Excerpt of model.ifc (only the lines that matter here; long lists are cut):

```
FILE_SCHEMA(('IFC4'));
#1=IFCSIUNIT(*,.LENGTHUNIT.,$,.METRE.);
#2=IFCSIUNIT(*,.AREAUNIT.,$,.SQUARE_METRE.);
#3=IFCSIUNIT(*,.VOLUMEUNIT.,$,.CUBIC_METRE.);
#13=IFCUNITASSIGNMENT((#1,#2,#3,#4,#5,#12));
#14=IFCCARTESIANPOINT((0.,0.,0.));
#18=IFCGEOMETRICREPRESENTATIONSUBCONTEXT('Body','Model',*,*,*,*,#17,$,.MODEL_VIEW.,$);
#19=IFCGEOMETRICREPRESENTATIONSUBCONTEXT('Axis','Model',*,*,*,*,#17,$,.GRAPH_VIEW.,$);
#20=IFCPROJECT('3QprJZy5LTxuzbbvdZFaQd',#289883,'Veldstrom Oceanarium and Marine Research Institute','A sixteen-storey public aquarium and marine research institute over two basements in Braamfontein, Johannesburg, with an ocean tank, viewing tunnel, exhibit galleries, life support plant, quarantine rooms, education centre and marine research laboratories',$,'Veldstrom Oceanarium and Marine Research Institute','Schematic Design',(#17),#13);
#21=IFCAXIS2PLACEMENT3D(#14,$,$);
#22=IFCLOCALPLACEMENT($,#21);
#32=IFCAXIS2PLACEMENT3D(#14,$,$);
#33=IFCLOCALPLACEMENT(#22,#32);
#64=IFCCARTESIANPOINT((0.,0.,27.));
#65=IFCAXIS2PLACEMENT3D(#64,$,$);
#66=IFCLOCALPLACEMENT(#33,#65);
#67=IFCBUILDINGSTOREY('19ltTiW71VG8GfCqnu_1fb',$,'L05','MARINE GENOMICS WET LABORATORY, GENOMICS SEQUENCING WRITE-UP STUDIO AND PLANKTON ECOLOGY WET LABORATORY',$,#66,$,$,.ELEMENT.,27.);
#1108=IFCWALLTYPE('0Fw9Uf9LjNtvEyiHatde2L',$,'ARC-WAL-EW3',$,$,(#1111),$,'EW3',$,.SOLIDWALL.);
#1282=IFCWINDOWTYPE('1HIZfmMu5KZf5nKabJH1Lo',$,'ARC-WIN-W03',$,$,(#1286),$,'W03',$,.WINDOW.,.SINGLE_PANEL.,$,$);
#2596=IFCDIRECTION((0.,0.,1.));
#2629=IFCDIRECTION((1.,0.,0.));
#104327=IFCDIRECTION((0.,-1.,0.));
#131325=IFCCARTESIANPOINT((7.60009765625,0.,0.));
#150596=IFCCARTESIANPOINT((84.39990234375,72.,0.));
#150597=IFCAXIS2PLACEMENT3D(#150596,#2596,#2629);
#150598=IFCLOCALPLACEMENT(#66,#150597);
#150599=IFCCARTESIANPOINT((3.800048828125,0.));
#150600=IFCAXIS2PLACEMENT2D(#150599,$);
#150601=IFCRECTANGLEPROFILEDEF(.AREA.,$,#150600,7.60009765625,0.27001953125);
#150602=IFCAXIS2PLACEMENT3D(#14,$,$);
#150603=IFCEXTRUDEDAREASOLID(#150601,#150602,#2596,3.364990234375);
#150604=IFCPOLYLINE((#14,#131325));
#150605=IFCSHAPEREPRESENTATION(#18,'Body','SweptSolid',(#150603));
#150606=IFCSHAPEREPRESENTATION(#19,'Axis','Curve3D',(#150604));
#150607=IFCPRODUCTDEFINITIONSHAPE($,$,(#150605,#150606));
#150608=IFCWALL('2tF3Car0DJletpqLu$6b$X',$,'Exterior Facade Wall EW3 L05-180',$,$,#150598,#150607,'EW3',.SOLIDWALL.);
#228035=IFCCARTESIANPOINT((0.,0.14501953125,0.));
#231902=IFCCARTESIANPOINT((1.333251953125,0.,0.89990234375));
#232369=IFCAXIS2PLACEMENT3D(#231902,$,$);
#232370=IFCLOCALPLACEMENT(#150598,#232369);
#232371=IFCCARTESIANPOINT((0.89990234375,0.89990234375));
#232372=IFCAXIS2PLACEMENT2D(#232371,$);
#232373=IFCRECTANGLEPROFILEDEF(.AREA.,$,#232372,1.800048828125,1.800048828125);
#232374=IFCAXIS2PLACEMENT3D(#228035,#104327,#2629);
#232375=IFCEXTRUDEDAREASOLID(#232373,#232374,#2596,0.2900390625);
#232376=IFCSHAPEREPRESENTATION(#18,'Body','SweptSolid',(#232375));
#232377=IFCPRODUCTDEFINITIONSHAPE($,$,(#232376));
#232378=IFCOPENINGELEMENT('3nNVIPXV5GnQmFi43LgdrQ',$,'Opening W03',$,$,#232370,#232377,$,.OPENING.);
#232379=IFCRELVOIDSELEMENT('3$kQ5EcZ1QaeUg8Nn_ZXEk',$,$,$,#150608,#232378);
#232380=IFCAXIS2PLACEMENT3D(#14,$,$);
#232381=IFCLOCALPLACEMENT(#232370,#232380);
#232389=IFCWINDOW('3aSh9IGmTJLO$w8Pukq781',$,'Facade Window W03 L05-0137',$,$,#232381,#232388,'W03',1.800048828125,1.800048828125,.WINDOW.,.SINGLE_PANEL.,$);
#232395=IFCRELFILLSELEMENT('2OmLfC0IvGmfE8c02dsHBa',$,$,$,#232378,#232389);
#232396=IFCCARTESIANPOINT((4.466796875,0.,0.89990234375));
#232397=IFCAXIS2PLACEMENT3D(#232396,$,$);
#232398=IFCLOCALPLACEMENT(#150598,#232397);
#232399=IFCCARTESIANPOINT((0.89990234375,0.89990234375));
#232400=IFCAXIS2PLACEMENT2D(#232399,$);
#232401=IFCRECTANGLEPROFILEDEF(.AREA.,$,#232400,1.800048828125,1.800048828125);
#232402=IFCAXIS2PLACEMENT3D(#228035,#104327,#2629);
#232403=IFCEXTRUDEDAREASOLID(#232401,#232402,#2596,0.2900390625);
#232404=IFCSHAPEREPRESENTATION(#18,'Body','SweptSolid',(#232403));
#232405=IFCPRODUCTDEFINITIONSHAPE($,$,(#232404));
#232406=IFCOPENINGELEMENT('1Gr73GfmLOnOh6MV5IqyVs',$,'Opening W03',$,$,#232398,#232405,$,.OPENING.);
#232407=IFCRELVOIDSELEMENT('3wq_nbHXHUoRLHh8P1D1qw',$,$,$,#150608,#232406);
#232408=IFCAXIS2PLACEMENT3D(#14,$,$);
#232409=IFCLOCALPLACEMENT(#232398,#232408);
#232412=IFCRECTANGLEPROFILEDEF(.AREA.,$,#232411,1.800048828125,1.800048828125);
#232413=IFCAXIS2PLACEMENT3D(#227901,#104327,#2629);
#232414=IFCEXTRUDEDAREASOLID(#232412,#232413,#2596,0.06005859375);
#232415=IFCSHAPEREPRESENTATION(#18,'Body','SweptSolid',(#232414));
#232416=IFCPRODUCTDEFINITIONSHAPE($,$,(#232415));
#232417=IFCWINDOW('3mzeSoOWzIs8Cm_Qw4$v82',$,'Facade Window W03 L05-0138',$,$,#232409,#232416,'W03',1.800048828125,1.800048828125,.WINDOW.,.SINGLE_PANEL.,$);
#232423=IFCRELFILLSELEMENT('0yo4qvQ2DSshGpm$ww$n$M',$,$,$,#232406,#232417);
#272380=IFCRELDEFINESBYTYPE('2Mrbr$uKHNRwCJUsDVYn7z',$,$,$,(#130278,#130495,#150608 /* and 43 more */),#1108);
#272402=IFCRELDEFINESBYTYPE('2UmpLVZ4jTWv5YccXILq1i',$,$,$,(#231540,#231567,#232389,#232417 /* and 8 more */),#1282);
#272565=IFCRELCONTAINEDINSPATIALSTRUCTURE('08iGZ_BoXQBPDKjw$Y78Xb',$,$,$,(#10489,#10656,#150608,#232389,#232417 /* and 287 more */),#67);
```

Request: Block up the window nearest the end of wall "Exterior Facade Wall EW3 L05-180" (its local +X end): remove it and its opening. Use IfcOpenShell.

```python
import ifcopenshell
import ifcopenshell.api.feature
import ifcopenshell.api.root
import ifcopenshell.geom
import ifcopenshell.util.shape

model = ifcopenshell.open("model.ifc")
settings = ifcopenshell.geom.settings()


def volume(element):
    """Net volume in cubic metres, openings subtracted."""
    shape = ifcopenshell.geom.create_shape(settings, element)
    return ifcopenshell.util.shape.get_volume(shape.geometry)


window = model.by_guid("3mzeSoOWzIs8Cm_Qw4$v82")
opening = window.FillsVoids[0].RelatingOpeningElement
wall = opening.VoidsElements[0].RelatingBuildingElement
before = volume(wall)

ifcopenshell.api.root.remove_product(model, product=window)
ifcopenshell.api.feature.remove_feature(model, feature=opening)

after = volume(wall)

print(f"wall volume {before:.3f} -> {after:.3f} m3")

model.write("model_rev.ifc")
```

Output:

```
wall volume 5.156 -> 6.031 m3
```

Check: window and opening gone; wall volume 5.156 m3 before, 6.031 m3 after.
